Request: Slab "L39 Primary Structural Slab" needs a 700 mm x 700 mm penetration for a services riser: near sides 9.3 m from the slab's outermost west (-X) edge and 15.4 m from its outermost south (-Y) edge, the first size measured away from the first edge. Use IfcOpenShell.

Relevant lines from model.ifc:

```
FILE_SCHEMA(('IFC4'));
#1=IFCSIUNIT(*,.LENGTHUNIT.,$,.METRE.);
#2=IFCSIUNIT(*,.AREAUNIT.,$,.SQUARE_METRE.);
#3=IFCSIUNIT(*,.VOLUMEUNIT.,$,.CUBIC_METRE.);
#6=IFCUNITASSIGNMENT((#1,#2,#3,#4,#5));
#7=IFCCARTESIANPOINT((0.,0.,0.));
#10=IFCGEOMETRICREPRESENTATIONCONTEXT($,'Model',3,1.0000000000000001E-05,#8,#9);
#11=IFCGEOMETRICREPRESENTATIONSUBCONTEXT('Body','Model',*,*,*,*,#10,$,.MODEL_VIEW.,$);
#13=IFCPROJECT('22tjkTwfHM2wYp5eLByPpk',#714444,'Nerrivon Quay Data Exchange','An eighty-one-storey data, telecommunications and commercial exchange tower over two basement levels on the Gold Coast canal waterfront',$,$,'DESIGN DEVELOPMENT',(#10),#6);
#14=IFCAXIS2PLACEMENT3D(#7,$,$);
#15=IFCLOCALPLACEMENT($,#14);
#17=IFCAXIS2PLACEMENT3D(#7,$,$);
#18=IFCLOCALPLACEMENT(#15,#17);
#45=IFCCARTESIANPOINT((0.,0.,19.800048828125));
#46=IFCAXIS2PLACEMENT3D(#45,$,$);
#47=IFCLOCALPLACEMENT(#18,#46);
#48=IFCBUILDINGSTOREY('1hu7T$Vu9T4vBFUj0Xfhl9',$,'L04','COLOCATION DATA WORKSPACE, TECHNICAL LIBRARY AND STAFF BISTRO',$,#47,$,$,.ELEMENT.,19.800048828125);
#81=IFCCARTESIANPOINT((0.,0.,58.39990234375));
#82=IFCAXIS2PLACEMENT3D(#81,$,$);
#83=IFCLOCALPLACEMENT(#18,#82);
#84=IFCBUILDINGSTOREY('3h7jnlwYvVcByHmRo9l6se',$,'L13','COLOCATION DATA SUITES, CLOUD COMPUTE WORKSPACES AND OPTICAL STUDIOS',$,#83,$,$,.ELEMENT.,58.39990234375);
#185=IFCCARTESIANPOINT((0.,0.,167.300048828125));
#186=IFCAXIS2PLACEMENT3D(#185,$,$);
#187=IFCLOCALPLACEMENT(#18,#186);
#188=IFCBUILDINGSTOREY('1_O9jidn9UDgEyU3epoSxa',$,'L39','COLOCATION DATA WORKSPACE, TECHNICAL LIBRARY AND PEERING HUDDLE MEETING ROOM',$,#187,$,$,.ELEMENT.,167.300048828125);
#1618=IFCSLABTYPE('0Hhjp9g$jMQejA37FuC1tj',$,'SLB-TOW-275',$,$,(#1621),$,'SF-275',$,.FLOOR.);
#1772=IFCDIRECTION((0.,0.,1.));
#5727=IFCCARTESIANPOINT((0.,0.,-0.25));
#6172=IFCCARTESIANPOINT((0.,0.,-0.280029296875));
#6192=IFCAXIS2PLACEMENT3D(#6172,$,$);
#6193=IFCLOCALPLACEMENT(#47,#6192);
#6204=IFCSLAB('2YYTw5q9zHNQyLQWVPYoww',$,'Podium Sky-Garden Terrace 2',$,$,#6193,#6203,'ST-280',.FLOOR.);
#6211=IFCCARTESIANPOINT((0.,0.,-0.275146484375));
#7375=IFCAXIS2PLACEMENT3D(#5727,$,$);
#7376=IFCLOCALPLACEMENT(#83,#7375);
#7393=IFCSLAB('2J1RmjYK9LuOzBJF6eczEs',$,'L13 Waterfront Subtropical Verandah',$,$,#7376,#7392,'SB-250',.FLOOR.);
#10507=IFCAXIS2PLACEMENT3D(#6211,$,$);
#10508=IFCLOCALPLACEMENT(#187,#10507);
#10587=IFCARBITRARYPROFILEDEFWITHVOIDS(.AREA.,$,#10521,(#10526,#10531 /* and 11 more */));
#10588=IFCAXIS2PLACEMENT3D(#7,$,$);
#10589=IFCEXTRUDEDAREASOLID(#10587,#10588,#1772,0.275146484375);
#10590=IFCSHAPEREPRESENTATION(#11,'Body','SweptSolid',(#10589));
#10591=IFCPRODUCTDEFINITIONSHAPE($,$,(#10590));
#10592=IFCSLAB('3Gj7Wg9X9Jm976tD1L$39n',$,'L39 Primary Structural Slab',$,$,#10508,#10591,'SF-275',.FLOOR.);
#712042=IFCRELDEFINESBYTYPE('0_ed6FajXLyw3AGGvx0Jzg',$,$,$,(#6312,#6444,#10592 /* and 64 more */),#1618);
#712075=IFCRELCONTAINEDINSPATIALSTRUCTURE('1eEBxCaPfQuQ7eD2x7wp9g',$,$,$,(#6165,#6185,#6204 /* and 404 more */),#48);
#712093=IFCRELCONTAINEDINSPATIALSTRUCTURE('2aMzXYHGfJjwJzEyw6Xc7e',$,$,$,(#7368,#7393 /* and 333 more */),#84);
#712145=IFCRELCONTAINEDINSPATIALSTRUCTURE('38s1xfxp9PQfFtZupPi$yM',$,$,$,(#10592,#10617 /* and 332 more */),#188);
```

```python
import numpy as np
import ifcopenshell
import ifcopenshell.api.feature
import ifcopenshell.api.geometry
import ifcopenshell.api.root
import ifcopenshell.geom
import ifcopenshell.util.placement
import ifcopenshell.util.representation
import ifcopenshell.util.shape
import ifcopenshell.util.unit

model = ifcopenshell.open("model.ifc")
unit_scale = ifcopenshell.util.unit.calculate_unit_scale(model)
settings = ifcopenshell.geom.settings()


def volume(element):
    """Net volume in cubic metres, openings subtracted."""
    shape = ifcopenshell.geom.create_shape(settings, element)
    return ifcopenshell.util.shape.get_volume(shape.geometry)


slab = model.by_guid("3Gj7Wg9X9Jm976tD1L$39n")
before = volume(slab)

# Extent in the slab's own axes, in metres. The edges named are its -X and -Y sides.
slab_shape = ifcopenshell.geom.create_shape(settings, slab)
vertices = ifcopenshell.util.shape.get_vertices(slab_shape.geometry)
x_min, y_min, bottom = vertices.min(axis=0)
top = vertices[:, 2].max()

opening = ifcopenshell.api.root.create_entity(model, ifc_class="IfcOpeningElement", name="Services riser opening", predefined_type="OPENING")
context = ifcopenshell.util.representation.get_context(model, "Model", "Body", "MODEL_VIEW")
width, depth = 0.7, 0.7
outline = [(0.0, 0.0), (width, 0.0), (width, depth), (0.0, depth), (0.0, 0.0)]
# Overshoot both faces by 50 mm so the cut is clean.
shape = ifcopenshell.api.geometry.add_slab_representation(
    model, context=context, depth=top - bottom + 0.1, polyline=outline
)
ifcopenshell.api.geometry.assign_representation(model, product=opening, representation=shape)

matrix = ifcopenshell.util.placement.get_local_placement(slab.ObjectPlacement)
matrix[:, 3] = matrix @ np.append(np.array([x_min + 9.3, y_min + 15.4, bottom - 0.05]) / unit_scale, 1.0)
ifcopenshell.api.geometry.edit_object_placement(model, product=opening, matrix=matrix, is_si=False)
ifcopenshell.api.feature.add_feature(model, feature=opening, element=slab)

after = volume(slab)

print(f"slab volume {before:.3f} -> {after:.3f} m3")

model.write("model_rev.ifc")
```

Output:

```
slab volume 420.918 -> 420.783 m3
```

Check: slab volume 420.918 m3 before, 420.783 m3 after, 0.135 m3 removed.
